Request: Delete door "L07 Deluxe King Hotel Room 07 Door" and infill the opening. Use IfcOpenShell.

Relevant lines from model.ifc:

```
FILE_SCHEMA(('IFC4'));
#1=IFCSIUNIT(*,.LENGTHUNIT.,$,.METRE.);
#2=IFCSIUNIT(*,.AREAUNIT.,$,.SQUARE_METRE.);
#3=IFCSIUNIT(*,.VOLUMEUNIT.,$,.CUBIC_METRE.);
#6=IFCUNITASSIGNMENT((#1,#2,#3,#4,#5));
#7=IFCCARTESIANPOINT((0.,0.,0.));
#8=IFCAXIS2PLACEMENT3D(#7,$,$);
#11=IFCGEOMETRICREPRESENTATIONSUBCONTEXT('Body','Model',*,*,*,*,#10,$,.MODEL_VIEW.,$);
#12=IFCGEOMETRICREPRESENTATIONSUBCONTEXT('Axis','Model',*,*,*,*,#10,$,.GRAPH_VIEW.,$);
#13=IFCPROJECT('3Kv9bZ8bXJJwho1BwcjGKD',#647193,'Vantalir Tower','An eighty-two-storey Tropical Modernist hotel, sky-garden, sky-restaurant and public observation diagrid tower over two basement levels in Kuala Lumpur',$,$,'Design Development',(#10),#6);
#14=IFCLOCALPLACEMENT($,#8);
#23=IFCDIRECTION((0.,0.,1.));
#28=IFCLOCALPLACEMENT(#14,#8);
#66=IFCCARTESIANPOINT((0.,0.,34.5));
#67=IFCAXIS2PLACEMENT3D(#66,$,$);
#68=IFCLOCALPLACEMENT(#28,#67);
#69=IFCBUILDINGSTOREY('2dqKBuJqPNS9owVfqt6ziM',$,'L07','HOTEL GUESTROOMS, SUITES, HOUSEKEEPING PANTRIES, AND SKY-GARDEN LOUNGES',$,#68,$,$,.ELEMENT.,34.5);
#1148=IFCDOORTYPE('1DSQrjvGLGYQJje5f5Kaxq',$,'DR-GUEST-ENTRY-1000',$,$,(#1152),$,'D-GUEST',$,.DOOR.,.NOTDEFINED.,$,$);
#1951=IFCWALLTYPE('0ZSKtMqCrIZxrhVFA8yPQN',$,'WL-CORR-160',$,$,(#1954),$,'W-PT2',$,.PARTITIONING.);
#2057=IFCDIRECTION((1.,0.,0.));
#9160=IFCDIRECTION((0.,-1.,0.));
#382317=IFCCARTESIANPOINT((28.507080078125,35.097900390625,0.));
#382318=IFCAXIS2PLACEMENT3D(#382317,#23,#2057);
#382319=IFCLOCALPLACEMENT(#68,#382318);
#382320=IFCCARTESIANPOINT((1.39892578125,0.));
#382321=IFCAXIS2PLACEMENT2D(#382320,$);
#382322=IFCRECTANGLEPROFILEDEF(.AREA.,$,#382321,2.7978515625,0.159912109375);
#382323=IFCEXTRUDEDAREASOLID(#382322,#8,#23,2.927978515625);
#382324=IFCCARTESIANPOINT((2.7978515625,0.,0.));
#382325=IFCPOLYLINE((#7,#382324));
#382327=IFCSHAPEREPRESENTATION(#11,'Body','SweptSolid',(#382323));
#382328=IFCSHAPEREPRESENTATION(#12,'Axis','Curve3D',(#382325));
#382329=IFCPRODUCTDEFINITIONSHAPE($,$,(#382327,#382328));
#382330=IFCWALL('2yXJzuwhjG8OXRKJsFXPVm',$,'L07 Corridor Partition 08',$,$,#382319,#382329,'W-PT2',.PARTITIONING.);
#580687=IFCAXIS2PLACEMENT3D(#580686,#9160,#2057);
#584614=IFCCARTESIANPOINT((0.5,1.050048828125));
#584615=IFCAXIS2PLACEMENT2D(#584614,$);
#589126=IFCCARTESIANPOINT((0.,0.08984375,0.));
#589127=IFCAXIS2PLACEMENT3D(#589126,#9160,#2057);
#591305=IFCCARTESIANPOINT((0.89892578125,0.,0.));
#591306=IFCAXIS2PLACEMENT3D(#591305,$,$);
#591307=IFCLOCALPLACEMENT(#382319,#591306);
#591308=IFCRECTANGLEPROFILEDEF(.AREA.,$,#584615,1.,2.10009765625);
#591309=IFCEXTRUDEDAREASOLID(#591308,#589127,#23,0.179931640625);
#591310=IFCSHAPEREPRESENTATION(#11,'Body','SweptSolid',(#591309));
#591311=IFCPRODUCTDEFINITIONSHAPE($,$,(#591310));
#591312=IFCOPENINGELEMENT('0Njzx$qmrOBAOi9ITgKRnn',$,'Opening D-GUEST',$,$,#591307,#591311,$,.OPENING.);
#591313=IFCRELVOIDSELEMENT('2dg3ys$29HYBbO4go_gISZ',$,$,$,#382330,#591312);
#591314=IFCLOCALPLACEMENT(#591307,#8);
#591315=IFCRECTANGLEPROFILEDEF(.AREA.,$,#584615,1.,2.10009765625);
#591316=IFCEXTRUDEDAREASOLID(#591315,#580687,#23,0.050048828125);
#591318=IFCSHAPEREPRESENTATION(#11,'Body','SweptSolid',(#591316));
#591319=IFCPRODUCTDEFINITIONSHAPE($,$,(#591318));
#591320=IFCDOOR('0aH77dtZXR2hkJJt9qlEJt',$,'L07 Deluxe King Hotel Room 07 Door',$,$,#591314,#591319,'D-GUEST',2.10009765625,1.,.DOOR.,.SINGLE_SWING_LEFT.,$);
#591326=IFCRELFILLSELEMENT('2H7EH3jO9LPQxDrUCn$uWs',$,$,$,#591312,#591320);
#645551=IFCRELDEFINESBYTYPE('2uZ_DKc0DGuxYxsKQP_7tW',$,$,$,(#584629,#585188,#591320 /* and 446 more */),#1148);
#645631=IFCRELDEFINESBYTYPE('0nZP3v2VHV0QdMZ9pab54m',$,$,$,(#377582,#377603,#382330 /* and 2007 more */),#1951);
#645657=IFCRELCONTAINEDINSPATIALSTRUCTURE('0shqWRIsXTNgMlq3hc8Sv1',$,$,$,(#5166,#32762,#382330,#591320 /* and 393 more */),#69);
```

```python
import ifcopenshell
import ifcopenshell.api.feature
import ifcopenshell.api.root
import ifcopenshell.geom
import ifcopenshell.util.shape

model = ifcopenshell.open("model.ifc")
settings = ifcopenshell.geom.settings()


def volume(element):
    """Net volume in cubic metres, openings subtracted."""
    shape = ifcopenshell.geom.create_shape(settings, element)
    return ifcopenshell.util.shape.get_volume(shape.geometry)


door = model.by_id(591320)
opening = door.FillsVoids[0].RelatingOpeningElement
wall = opening.VoidsElements[0].RelatingBuildingElement
before = volume(wall)

ifcopenshell.api.root.remove_product(model, product=door)
ifcopenshell.api.feature.remove_feature(model, feature=opening)

after = volume(wall)

print(f"wall volume {before:.3f} -> {after:.3f} m3")

model.write("model-out.ifc")
```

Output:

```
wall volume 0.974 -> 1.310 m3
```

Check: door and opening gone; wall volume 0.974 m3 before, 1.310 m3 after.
